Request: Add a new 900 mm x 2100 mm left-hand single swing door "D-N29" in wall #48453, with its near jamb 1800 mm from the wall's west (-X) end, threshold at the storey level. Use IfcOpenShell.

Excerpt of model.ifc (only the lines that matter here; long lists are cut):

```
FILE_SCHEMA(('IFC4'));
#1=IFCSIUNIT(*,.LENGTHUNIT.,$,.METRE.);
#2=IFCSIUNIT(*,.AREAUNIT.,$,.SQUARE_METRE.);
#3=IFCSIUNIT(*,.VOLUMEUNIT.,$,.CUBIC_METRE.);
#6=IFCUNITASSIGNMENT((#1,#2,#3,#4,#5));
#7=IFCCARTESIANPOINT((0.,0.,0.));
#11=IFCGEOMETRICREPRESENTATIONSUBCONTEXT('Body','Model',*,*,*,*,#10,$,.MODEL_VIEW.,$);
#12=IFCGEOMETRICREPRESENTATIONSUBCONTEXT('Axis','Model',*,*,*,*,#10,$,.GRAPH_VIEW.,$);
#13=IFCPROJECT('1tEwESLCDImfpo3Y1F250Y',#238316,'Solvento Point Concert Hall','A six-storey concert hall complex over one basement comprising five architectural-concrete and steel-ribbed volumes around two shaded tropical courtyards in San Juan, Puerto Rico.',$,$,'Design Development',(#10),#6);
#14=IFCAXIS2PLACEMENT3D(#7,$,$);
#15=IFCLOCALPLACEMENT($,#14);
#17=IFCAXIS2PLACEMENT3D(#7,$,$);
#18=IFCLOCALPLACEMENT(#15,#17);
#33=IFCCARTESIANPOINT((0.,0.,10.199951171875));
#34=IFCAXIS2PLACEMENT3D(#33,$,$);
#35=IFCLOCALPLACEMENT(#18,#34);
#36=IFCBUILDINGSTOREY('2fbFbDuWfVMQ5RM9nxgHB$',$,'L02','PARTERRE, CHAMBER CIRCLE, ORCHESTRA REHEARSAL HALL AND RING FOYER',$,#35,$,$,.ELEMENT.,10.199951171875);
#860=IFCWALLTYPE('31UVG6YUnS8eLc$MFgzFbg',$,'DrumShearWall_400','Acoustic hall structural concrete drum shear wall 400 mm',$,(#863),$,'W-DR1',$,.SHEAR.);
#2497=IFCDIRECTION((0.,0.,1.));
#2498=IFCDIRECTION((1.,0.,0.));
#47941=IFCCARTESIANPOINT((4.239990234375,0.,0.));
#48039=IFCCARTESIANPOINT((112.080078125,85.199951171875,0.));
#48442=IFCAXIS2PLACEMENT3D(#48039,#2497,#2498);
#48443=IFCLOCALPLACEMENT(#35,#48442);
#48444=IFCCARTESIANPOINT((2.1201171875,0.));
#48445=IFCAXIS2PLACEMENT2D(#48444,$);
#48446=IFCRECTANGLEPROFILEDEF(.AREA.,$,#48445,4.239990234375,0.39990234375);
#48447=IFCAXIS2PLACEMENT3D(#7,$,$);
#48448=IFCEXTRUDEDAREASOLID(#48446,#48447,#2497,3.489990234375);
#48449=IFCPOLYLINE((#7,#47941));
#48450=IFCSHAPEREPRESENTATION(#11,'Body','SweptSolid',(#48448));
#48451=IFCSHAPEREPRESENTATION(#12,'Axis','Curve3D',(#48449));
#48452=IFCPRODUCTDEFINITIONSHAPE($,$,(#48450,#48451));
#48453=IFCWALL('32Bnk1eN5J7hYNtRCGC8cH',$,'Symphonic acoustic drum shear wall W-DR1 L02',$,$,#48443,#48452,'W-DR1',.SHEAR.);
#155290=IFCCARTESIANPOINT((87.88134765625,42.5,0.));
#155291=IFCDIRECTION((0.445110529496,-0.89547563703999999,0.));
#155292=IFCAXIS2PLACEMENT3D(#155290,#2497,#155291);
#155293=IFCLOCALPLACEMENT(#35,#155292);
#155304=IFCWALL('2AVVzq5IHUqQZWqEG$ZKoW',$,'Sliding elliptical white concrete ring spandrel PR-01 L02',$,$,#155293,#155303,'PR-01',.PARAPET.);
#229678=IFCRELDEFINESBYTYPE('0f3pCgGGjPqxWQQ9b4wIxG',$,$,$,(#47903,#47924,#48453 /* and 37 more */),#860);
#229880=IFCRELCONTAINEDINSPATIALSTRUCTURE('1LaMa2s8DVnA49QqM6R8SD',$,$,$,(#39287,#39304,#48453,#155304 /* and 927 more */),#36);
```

```python
import numpy as np
import ifcopenshell
import ifcopenshell.api.feature
import ifcopenshell.api.geometry
import ifcopenshell.api.root
import ifcopenshell.api.spatial
import ifcopenshell.geom
import ifcopenshell.util.element
import ifcopenshell.util.placement
import ifcopenshell.util.representation
import ifcopenshell.util.shape
import ifcopenshell.util.unit

model = ifcopenshell.open("model.ifc")
unit_scale = ifcopenshell.util.unit.calculate_unit_scale(model)
settings = ifcopenshell.geom.settings()


def volume(element):
    """Net volume in cubic metres, openings subtracted."""
    shape = ifcopenshell.geom.create_shape(settings, element)
    return ifcopenshell.util.shape.get_volume(shape.geometry)


wall = model.by_id(48453)
storey = ifcopenshell.util.element.get_container(wall, ifc_class="IfcBuildingStorey")
context = ifcopenshell.util.representation.get_context(model, "Model", "Body", "MODEL_VIEW")
before = volume(wall)

width, height, from_end, sill = 0.9, 2.1, 1.8, 0.0  # metres

# The wall runs along its own X axis, and the end named is its -X end.
wall_shape = ifcopenshell.geom.create_shape(settings, wall)
x, y, z = ifcopenshell.util.shape.get_vertices(wall_shape.geometry).T
start = x.min() + from_end
face, thickness = float(y.min()), float(y.max() - y.min())
wall_matrix = ifcopenshell.util.placement.get_local_placement(wall.ObjectPlacement)
level = ifcopenshell.util.placement.get_local_placement(storey.ObjectPlacement)[2, 3]


def in_wall(x, y):
    """Placement at x, y metres in the wall's axes, at sill height."""
    matrix = wall_matrix.copy()
    matrix[:, 3] = wall_matrix @ np.array([x / unit_scale, y / unit_scale, 0.0, 1.0])
    matrix[2, 3] = level + sill / unit_scale
    return matrix


# Opening: a box that overshoots both wall faces by 50 mm.
opening = ifcopenshell.api.root.create_entity(model, ifc_class="IfcOpeningElement", predefined_type="OPENING")
box = ifcopenshell.api.geometry.add_wall_representation(
    model, context=context, length=width, height=height, thickness=thickness + 0.1
)
ifcopenshell.api.geometry.assign_representation(model, product=opening, representation=box)
ifcopenshell.api.geometry.edit_object_placement(model, product=opening, matrix=in_wall(start, face - 0.05), is_si=False)
ifcopenshell.api.feature.add_feature(model, feature=opening, element=wall)

door = ifcopenshell.api.root.create_entity(model, ifc_class="IfcDoor", name="D-N29", predefined_type="DOOR")
door.OverallWidth, door.OverallHeight = width / unit_scale, height / unit_scale
door.OperationType = "SINGLE_SWING_LEFT"
body = ifcopenshell.api.geometry.add_door_representation(
    model,
    context=context,
    overall_width=door.OverallWidth,
    overall_height=door.OverallHeight,
    operation_type="SINGLE_SWING_LEFT",
    lining_properties={"LiningDepth": thickness / unit_scale, "ThresholdDepth": thickness / unit_scale},
)
ifcopenshell.api.geometry.assign_representation(model, product=door, representation=body)
ifcopenshell.api.spatial.assign_container(model, products=[door], relating_structure=storey)
ifcopenshell.api.feature.add_filling(model, opening=opening, element=door)

# The lining spans the wall, so the door starts at the wall face.
ifcopenshell.api.geometry.edit_object_placement(model, product=door, matrix=in_wall(start, face), is_si=False)

after = volume(wall)

print(f"wall volume {before:.3f} -> {after:.3f} m3")

model.write("model_updated.ifc")
```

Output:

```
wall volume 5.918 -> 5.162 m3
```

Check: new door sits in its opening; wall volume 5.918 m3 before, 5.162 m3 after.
